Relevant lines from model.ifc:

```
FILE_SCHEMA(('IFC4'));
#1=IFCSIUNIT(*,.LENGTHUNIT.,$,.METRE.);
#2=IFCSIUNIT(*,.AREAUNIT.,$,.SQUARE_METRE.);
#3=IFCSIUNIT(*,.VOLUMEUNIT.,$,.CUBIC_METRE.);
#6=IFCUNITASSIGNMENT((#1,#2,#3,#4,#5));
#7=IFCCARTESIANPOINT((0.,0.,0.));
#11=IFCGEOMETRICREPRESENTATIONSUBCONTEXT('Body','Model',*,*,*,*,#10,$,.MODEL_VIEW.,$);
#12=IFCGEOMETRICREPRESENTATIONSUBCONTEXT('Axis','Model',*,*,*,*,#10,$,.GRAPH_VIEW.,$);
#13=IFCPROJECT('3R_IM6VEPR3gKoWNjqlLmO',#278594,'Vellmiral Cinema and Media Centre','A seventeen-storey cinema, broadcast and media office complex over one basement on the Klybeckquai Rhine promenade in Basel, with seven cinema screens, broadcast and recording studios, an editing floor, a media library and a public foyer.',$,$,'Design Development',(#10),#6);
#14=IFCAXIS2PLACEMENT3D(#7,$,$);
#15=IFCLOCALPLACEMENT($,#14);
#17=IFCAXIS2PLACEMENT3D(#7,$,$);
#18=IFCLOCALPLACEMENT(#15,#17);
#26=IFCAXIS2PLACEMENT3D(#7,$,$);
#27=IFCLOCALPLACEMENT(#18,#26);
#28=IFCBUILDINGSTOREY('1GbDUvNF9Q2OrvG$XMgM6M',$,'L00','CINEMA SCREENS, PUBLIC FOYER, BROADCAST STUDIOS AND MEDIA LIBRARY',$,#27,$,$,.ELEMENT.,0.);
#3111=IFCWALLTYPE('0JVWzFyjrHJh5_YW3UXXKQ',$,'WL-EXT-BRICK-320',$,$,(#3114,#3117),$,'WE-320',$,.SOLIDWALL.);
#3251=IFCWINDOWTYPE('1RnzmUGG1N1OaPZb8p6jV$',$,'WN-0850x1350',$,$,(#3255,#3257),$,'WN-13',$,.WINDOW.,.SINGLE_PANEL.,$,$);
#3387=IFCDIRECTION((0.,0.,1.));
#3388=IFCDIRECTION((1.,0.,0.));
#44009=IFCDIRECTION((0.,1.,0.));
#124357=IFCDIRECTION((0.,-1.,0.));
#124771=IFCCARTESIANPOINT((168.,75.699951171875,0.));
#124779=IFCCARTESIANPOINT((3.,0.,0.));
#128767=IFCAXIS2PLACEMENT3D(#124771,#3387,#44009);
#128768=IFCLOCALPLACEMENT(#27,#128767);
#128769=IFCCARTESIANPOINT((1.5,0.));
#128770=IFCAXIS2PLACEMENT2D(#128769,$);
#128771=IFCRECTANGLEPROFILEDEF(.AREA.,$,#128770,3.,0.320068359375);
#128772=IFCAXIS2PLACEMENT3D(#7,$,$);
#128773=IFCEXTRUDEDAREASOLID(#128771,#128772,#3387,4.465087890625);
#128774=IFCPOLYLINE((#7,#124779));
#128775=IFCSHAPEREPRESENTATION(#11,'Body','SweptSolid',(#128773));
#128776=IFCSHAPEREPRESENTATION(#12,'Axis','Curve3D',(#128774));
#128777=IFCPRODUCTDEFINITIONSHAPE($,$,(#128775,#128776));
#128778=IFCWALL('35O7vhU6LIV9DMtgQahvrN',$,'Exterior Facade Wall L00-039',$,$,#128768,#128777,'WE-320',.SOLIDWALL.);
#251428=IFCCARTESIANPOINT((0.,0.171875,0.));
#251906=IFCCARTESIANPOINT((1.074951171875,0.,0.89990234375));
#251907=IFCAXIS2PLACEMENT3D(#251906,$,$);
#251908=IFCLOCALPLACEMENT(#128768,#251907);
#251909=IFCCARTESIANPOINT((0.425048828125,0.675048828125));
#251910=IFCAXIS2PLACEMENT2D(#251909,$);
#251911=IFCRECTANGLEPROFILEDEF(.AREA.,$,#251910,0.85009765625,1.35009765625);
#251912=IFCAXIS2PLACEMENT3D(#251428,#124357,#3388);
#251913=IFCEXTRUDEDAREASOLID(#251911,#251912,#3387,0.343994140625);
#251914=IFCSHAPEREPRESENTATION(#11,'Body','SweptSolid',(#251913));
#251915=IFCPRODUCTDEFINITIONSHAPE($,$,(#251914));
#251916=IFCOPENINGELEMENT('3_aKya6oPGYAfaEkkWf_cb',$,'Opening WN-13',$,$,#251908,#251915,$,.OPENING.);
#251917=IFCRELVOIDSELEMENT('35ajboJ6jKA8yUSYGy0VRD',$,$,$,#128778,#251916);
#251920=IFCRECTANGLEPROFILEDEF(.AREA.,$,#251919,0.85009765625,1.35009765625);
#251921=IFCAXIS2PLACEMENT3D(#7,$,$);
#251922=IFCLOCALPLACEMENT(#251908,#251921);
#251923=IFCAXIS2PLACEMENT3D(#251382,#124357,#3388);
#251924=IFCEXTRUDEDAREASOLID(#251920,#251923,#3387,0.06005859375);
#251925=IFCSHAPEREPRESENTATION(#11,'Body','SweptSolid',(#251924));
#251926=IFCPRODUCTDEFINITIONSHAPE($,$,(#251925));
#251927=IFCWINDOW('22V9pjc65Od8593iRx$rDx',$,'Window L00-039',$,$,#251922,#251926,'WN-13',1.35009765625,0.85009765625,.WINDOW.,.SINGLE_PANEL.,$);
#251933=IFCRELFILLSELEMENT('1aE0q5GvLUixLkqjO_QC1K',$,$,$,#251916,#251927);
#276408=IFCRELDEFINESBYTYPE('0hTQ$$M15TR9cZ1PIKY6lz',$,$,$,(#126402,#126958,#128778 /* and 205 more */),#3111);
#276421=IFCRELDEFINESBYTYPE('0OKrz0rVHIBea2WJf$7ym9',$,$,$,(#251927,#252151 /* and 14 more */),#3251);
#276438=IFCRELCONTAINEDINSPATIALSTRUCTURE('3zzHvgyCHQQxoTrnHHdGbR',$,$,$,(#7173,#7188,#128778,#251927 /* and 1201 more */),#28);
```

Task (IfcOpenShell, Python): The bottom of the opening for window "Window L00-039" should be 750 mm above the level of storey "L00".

```python
import numpy as np
import ifcopenshell
import ifcopenshell.api.geometry
import ifcopenshell.geom
import ifcopenshell.util.element
import ifcopenshell.util.placement
import ifcopenshell.util.shape
import ifcopenshell.util.unit

model = ifcopenshell.open("model.ifc")
unit_scale = ifcopenshell.util.unit.calculate_unit_scale(model)

window = model.by_guid("22V9pjc65Od8593iRx$rDx")
opening = window.FillsVoids[0].RelatingOpeningElement
storey = ifcopenshell.util.element.get_container(window, ifc_class="IfcBuildingStorey")
level = ifcopenshell.util.placement.get_local_placement(storey.ObjectPlacement)[2, 3]

# The opening's origin need not be at the sill, so measure its lowest point.
shape = ifcopenshell.geom.create_shape(ifcopenshell.geom.settings(), opening)
bottom = ifcopenshell.util.shape.get_shape_bottom_elevation(shape, shape.geometry) / unit_scale
dz = level + 0.75 / unit_scale - bottom

shift = np.array([0.0, 0.0, dz])
# The window is placed relative to its opening, so it follows when the opening moves.
matrix = ifcopenshell.util.placement.get_local_placement(opening.ObjectPlacement)
matrix[:3, 3] += shift
ifcopenshell.api.geometry.edit_object_placement(
    model, product=opening, matrix=matrix, is_si=False, should_transform_children=True
)

print(f"moved by {dz * unit_scale:+.3f} m")

model.write("model-out.ifc")
```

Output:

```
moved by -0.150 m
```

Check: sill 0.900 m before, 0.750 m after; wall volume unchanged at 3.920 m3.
